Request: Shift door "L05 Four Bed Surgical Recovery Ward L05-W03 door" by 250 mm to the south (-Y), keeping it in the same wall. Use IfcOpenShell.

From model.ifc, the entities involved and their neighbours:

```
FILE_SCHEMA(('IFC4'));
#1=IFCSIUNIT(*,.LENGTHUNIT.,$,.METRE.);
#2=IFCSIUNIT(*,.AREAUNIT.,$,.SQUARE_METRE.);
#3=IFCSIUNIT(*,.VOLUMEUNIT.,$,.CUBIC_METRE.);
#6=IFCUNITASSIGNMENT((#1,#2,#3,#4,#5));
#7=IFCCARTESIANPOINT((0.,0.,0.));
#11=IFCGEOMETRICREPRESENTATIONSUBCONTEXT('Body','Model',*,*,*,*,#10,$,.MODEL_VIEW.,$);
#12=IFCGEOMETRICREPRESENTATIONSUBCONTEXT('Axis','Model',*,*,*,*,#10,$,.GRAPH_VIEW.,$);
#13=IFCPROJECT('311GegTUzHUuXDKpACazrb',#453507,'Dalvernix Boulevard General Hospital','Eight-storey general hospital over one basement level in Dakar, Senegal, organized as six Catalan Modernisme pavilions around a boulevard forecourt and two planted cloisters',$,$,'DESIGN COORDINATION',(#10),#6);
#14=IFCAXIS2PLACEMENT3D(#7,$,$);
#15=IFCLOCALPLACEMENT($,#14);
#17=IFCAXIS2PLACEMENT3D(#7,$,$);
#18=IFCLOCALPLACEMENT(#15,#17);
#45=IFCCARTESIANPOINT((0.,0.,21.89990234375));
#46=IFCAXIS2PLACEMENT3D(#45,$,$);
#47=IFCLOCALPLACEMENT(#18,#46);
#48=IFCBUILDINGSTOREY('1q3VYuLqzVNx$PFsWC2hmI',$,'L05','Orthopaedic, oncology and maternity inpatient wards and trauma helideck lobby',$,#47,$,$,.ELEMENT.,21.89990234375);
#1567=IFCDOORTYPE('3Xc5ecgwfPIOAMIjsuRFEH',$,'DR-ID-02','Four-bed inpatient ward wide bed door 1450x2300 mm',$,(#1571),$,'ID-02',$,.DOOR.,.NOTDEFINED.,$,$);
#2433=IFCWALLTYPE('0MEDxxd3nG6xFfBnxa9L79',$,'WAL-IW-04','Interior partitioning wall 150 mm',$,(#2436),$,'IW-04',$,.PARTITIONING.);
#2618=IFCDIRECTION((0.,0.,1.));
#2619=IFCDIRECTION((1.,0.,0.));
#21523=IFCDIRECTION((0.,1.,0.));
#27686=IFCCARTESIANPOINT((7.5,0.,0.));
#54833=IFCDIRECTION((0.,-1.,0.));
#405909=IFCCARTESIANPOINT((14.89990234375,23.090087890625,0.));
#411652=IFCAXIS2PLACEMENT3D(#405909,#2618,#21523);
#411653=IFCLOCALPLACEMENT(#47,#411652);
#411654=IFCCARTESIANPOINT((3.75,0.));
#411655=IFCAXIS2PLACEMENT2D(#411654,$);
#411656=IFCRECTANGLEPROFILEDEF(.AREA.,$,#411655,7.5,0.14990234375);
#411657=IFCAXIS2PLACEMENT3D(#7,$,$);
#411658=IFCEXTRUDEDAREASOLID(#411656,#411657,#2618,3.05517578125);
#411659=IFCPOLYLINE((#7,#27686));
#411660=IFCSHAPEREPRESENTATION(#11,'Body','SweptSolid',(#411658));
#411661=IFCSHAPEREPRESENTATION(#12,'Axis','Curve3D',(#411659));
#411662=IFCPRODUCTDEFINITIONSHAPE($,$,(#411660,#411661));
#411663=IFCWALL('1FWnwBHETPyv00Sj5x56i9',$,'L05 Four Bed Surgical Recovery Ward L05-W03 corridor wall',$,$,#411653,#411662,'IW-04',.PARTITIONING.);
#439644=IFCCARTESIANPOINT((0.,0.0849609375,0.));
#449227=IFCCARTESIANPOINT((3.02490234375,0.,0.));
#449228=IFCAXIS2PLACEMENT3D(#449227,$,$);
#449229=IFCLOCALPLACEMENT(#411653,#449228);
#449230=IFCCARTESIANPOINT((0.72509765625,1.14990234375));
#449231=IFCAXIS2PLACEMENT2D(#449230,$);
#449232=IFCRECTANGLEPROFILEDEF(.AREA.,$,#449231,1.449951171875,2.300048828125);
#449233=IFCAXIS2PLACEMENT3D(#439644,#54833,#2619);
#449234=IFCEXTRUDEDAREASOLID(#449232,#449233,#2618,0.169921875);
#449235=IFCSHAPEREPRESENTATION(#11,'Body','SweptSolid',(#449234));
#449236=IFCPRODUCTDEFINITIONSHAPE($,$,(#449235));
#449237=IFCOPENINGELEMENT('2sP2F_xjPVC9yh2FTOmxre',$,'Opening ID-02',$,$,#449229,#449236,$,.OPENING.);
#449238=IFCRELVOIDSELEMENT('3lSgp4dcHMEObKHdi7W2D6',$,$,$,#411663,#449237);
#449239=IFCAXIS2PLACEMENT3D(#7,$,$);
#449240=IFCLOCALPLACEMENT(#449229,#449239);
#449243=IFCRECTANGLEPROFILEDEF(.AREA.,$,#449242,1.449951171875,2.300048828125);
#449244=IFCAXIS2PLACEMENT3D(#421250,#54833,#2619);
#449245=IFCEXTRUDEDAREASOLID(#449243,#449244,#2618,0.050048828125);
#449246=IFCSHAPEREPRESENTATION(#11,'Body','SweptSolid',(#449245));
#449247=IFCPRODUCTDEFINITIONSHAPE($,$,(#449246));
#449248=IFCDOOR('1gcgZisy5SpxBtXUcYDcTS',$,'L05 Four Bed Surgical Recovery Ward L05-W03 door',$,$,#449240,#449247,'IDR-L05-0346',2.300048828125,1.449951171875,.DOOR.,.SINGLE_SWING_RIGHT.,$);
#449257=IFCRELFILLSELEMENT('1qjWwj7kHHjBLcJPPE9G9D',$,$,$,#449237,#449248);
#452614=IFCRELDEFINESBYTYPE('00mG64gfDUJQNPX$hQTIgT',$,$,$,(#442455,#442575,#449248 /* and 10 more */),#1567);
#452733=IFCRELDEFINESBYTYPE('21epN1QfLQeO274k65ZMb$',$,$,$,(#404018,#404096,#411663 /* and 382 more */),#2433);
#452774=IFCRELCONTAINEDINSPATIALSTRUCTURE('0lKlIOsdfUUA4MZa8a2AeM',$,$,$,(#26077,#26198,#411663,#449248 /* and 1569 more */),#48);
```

```python
import ifcopenshell
import ifcopenshell.api.geometry
import ifcopenshell.util.placement

model = ifcopenshell.open("model.ifc")

door = model.by_id(449248)
opening = door.FillsVoids[0].RelatingOpeningElement
wall = opening.VoidsElements[0].RelatingBuildingElement

wall_matrix = ifcopenshell.util.placement.get_local_placement(wall.ObjectPlacement)
shift = wall_matrix[:3, 0] * -0.25
before = ifcopenshell.util.placement.get_local_placement(door.ObjectPlacement)[:3, 3].copy()

# The door is placed relative to its opening, so it follows when the opening moves.
matrix = ifcopenshell.util.placement.get_local_placement(opening.ObjectPlacement)
matrix[:3, 3] += shift
ifcopenshell.api.geometry.edit_object_placement(
    model, product=opening, matrix=matrix, is_si=False, should_transform_children=True
)

after = ifcopenshell.util.placement.get_local_placement(door.ObjectPlacement)[:3, 3]
print("door moved by", (after - before).round(3) + 0.0)

model.write("model_updated.ifc")
```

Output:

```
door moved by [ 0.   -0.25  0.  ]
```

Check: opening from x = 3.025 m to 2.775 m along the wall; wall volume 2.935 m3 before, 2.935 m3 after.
